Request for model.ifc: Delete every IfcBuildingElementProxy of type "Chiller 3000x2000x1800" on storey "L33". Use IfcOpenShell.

First a look at what the model holds.

```python
import ifcopenshell
import ifcopenshell.util.element

model = ifcopenshell.open("model.ifc")
print(model.schema)
storey = next(s for s in model.by_type("IfcBuildingStorey") if s.Name == "L33")
proxies = [e for e in ifcopenshell.util.element.get_decomposition(storey) if e.is_a("IfcBuildingElementProxy")]
seen = {}
for e in proxies:
    element_type = ifcopenshell.util.element.get_type(e)
    name = element_type.Name if element_type not in (None, e) else None
    seen[name] = seen.get(name, 0) + 1
for name, count in sorted(seen.items(), key=str):
    print(count, "x", name)
```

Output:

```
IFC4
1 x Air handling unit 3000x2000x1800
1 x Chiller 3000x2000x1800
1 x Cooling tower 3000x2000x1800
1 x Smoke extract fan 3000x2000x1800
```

```python
import ifcopenshell
import ifcopenshell.api.root
import ifcopenshell.util.element

model = ifcopenshell.open("model.ifc")

storey = next(s for s in model.by_type("IfcBuildingStorey") if s.Name == "L33")
proxies = [e for e in ifcopenshell.util.element.get_decomposition(storey) if e.is_a("IfcBuildingElementProxy")]
targets = [e for e in proxies if (t := ifcopenshell.util.element.get_type(e)) not in (None, e) and t.Name == "Chiller 3000x2000x1800"]

for e in targets:
    ifcopenshell.api.root.remove_product(model, product=e)
print(len(targets), "removed")

model.write("model_updated.ifc")
```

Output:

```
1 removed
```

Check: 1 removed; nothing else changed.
